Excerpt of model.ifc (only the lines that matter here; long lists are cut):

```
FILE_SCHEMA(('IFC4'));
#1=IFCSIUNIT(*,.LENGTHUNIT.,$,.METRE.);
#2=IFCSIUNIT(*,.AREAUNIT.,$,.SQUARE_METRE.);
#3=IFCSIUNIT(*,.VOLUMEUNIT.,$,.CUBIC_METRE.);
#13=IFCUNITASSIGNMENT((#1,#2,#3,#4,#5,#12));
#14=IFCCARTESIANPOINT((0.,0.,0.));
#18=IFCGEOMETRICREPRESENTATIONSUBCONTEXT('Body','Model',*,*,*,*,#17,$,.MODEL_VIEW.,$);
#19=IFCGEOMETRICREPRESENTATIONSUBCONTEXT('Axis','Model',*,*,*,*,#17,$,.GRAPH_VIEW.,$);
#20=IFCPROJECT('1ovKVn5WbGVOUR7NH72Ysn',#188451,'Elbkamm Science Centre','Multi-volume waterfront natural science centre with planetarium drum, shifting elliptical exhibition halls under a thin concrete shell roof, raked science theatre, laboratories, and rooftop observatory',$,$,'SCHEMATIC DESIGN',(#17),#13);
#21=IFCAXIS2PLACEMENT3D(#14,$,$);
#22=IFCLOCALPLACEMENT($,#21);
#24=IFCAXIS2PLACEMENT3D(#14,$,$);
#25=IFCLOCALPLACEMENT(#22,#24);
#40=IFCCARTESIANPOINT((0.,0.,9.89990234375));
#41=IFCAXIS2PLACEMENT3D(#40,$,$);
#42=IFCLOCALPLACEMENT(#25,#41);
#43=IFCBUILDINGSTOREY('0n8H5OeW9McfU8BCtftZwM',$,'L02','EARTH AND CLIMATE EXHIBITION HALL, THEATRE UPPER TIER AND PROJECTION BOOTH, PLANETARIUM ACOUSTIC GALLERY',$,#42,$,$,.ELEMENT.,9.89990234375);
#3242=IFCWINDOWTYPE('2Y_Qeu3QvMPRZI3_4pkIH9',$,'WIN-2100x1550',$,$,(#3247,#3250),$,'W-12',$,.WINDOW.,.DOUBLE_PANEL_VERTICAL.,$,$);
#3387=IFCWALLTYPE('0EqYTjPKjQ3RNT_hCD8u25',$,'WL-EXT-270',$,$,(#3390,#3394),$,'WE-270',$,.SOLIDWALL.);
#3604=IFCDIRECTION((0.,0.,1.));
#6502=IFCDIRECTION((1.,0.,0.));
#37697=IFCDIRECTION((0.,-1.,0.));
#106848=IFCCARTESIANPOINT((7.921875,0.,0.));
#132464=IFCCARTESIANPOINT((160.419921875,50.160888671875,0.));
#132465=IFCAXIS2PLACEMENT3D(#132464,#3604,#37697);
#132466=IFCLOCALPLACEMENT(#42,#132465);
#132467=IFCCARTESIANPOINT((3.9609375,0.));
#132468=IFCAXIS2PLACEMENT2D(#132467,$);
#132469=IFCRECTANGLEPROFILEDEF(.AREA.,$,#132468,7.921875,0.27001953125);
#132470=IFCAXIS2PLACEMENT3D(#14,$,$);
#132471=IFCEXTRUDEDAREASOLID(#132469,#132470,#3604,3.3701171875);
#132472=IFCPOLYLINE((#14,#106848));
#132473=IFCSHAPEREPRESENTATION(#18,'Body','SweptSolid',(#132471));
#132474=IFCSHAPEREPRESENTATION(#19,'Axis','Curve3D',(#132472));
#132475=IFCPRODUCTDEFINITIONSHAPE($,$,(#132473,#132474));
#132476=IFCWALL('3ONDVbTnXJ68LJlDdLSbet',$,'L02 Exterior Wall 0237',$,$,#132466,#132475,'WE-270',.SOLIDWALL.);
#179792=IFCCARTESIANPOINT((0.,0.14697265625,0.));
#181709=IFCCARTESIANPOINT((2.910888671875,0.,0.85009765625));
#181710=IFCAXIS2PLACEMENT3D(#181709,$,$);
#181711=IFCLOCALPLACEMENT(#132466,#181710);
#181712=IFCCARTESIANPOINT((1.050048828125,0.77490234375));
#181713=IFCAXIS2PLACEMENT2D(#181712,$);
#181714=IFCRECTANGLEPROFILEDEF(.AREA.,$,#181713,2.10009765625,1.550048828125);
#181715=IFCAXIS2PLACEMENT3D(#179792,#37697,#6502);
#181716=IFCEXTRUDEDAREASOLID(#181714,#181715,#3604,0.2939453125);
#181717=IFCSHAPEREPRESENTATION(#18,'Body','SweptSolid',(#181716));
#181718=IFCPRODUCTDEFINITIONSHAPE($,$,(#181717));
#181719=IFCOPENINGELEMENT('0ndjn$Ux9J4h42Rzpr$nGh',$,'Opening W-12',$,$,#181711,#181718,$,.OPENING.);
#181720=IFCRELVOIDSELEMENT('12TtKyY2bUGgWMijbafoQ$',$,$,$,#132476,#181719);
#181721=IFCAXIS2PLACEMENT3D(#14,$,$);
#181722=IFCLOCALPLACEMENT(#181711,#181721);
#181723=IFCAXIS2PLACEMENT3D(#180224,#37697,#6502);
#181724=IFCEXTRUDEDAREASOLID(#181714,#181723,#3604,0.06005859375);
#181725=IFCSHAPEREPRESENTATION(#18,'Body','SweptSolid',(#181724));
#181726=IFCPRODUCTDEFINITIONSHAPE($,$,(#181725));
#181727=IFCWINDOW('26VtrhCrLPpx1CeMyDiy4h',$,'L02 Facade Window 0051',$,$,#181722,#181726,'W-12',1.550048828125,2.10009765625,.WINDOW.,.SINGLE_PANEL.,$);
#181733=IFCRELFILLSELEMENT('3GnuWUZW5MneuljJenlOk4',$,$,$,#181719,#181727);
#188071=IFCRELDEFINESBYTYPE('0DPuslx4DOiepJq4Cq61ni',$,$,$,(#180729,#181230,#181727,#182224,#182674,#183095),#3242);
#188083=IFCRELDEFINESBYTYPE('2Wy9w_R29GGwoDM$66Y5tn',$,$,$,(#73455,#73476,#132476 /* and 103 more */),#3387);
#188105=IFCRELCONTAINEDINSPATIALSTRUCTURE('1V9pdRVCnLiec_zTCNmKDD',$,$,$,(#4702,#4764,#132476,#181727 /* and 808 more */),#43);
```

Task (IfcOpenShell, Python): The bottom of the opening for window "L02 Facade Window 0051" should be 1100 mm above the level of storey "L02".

```python
import numpy as np
import ifcopenshell
import ifcopenshell.api.geometry
import ifcopenshell.geom
import ifcopenshell.util.element
import ifcopenshell.util.placement
import ifcopenshell.util.shape
import ifcopenshell.util.unit

model = ifcopenshell.open("model.ifc")
unit_scale = ifcopenshell.util.unit.calculate_unit_scale(model)

window = model.by_guid("26VtrhCrLPpx1CeMyDiy4h")
opening = window.FillsVoids[0].RelatingOpeningElement
storey = ifcopenshell.util.element.get_container(window, ifc_class="IfcBuildingStorey")
level = ifcopenshell.util.placement.get_local_placement(storey.ObjectPlacement)[2, 3]

# The opening's origin need not be at the sill, so measure its lowest point.
shape = ifcopenshell.geom.create_shape(ifcopenshell.geom.settings(), opening)
bottom = ifcopenshell.util.shape.get_shape_bottom_elevation(shape, shape.geometry) / unit_scale
dz = level + 1.1 - bottom

shift = np.array([0.0, 0.0, dz])
# The window is placed relative to its opening, so it follows when the opening moves.
matrix = ifcopenshell.util.placement.get_local_placement(opening.ObjectPlacement)
matrix[:3, 3] += shift
ifcopenshell.api.geometry.edit_object_placement(
    model, product=opening, matrix=matrix, is_si=False, should_transform_children=True
)

print(f"moved by {dz * unit_scale:+.3f} m")

model.write("model_v2.ifc")
```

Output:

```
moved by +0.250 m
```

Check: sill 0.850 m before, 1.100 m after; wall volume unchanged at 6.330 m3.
